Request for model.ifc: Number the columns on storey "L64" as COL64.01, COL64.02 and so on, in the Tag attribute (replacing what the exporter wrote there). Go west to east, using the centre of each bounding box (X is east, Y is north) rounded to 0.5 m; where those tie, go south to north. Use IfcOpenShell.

First a look at what the model holds.

```python
import ifcopenshell
import ifcopenshell.util.element
import ifcopenshell.util.placement

model = ifcopenshell.open("model.ifc")
print(model.schema)
storey = next(s for s in model.by_type("IfcBuildingStorey") if s.Name == "L64")
columns = [e for e in ifcopenshell.util.element.get_decomposition(storey) if e.is_a("IfcColumn")]
for e in sorted(columns, key=lambda e: e.id()):
    origin = ifcopenshell.util.placement.get_local_placement(e.ObjectPlacement)[:3, 3]
    print(e.id(), e.Tag, e.Name, origin.round(2) + 0.0, sep=" | ")
```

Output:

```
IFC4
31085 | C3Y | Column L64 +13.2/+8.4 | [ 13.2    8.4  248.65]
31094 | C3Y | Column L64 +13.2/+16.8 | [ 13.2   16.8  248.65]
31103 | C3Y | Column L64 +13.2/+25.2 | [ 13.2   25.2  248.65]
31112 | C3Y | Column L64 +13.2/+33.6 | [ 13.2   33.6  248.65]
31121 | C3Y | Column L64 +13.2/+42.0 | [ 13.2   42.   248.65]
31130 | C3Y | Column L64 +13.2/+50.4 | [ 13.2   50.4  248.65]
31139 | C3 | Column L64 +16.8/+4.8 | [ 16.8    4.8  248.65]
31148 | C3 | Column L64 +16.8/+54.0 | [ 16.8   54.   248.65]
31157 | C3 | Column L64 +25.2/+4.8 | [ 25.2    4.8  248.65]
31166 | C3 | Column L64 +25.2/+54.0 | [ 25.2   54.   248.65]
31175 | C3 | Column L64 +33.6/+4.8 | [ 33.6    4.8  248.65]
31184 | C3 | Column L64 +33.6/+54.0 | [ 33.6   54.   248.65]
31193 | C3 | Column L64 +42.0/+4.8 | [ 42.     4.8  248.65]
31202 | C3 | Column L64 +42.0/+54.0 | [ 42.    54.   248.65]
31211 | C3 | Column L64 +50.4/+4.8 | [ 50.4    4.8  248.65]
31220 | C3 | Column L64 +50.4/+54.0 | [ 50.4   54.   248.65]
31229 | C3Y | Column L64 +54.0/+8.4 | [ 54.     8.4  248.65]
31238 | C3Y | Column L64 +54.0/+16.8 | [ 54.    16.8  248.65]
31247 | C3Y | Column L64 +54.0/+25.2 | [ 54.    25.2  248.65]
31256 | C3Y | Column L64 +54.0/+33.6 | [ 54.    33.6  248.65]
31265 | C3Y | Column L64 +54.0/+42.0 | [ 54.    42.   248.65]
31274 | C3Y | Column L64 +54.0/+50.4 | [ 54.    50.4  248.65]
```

```python
import ifcopenshell
import ifcopenshell.geom
import ifcopenshell.util.element
import ifcopenshell.util.shape

model = ifcopenshell.open("model.ifc")
settings = ifcopenshell.geom.settings()
settings.set("use-world-coords", True)


def centre(element):
    shape = ifcopenshell.geom.create_shape(settings, element)
    return ifcopenshell.util.shape.get_bbox_centroid(shape.geometry)


storey = next(s for s in model.by_type("IfcBuildingStorey") if s.Name == "L64")
columns = [e for e in ifcopenshell.util.element.get_decomposition(storey) if e.is_a("IfcColumn")]

# Insertion points can sit at a corner or the storey origin, so sort by the geometry (in metres).
centres = {e: centre(e) for e in columns}
columns.sort(key=lambda e: (round(centres[e][0] / 0.5), centres[e][1]))

for i, e in enumerate(columns, start=1):
    number = f"COL64.{i:02d}"
    e.Tag = number
    print(e.id(), number)

model.write("model_rev.ifc")
```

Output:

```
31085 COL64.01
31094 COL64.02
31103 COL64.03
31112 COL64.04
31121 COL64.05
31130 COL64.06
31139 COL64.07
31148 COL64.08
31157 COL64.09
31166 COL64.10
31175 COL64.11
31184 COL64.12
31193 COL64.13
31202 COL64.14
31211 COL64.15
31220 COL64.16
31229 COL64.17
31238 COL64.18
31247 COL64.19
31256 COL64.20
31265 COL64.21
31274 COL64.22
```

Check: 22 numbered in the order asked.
